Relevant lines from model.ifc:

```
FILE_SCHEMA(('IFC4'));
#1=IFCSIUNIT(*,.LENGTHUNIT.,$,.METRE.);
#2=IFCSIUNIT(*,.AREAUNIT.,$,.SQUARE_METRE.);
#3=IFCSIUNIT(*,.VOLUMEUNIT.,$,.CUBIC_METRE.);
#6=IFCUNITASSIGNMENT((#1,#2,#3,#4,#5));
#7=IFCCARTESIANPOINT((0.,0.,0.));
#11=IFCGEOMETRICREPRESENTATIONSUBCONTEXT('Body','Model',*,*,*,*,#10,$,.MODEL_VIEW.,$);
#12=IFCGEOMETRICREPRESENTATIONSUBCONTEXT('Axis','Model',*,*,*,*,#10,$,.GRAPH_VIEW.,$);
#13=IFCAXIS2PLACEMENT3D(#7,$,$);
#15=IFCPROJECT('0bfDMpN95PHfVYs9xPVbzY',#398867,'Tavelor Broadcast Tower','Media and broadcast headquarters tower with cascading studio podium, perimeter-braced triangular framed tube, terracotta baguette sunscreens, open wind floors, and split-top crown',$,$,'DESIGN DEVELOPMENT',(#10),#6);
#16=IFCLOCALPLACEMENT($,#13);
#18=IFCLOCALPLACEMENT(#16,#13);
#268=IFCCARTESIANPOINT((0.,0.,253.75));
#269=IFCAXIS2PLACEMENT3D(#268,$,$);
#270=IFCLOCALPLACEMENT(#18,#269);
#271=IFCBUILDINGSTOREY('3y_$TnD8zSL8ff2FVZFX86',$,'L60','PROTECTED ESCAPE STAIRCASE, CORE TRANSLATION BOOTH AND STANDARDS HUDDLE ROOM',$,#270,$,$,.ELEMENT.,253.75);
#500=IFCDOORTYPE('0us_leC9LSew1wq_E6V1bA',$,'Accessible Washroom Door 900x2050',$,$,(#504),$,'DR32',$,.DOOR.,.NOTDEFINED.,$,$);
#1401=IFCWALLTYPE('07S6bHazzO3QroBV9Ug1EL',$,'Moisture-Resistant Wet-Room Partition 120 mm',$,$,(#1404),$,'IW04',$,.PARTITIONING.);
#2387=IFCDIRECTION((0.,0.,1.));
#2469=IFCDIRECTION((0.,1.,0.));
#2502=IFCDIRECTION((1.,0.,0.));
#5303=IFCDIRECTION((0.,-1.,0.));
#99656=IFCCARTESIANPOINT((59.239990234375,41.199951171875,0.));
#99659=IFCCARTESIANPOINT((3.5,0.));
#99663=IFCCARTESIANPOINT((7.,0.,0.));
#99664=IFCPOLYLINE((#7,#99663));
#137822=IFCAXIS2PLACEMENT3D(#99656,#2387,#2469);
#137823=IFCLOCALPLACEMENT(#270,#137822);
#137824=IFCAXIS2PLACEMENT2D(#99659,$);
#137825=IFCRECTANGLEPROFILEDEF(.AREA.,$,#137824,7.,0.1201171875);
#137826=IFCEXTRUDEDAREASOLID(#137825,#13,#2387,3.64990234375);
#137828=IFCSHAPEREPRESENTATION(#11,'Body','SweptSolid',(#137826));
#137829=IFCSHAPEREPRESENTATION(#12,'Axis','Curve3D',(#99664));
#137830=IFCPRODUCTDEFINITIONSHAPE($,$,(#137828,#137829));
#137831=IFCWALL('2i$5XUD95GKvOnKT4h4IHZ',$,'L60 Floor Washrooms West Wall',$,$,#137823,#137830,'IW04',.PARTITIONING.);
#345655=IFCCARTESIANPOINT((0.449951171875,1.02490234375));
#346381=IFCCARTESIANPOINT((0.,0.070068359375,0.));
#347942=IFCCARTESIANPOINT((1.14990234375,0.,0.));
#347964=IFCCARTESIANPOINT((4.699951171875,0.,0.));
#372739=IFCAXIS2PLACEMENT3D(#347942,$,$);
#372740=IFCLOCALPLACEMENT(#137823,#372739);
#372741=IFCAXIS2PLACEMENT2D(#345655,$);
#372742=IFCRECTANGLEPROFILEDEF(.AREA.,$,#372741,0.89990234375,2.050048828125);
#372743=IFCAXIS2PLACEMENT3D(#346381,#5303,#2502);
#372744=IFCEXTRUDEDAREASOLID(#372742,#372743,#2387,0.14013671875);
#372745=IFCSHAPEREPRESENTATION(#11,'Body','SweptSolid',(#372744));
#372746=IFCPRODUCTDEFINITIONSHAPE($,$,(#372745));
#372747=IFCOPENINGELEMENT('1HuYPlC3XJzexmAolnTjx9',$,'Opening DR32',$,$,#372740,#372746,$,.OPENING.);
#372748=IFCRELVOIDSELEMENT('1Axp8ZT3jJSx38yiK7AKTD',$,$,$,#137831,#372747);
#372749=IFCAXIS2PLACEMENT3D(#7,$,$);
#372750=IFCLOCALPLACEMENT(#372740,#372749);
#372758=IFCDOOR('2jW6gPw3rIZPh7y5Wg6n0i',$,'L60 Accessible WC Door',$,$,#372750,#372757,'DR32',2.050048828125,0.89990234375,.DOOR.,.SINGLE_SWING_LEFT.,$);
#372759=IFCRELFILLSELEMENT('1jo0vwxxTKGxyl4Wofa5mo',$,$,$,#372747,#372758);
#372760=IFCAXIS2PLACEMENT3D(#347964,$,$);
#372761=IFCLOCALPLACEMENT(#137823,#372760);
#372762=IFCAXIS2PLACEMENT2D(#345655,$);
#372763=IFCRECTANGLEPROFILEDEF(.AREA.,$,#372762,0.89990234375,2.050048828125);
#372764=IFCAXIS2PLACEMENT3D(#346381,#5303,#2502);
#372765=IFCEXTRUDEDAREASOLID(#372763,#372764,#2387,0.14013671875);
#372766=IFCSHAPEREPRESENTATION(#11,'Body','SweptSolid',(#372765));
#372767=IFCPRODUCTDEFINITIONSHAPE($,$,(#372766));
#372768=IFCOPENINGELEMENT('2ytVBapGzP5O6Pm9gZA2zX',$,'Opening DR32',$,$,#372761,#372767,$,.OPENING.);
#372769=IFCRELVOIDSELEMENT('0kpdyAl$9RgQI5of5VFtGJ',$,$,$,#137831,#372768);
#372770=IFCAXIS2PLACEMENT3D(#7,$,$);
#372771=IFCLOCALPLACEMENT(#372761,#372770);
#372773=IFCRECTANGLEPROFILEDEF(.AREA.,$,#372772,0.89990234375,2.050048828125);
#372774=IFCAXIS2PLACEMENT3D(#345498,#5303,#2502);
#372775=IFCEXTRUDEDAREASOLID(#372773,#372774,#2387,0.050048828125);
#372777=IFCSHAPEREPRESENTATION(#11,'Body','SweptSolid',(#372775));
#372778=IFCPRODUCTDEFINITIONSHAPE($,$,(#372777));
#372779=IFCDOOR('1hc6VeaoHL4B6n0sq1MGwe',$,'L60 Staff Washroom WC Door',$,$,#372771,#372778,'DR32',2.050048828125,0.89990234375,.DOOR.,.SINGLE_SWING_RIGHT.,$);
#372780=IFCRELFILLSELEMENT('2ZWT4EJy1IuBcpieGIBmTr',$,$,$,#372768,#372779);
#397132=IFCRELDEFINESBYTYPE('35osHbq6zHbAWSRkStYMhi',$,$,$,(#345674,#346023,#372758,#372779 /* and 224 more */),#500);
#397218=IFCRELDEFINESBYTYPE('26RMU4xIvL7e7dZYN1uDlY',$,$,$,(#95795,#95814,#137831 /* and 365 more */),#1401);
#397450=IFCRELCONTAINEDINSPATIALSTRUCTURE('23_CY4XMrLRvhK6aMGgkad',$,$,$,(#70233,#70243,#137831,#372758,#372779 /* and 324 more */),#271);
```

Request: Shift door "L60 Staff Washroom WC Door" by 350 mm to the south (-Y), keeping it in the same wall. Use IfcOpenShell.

```python
import ifcopenshell
import ifcopenshell.api.geometry
import ifcopenshell.util.placement
import ifcopenshell.util.unit

model = ifcopenshell.open("model.ifc")
unit_scale = ifcopenshell.util.unit.calculate_unit_scale(model)

door = model.by_guid("1hc6VeaoHL4B6n0sq1MGwe")
opening = door.FillsVoids[0].RelatingOpeningElement
wall = opening.VoidsElements[0].RelatingBuildingElement

wall_matrix = ifcopenshell.util.placement.get_local_placement(wall.ObjectPlacement)
shift = wall_matrix[:3, 0] * -0.35 / unit_scale
before = ifcopenshell.util.placement.get_local_placement(door.ObjectPlacement)[:3, 3].copy()

# The door is placed relative to its opening, so it follows when the opening moves.
matrix = ifcopenshell.util.placement.get_local_placement(opening.ObjectPlacement)
matrix[:3, 3] += shift
ifcopenshell.api.geometry.edit_object_placement(
    model, product=opening, matrix=matrix, is_si=False, should_transform_children=True
)

after = ifcopenshell.util.placement.get_local_placement(door.ObjectPlacement)[:3, 3]
print("door moved by", (after - before).round(3) + 0.0)

model.write("model_updated.ifc")
```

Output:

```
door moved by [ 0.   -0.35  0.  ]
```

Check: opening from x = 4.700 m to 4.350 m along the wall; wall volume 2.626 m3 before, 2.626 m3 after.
